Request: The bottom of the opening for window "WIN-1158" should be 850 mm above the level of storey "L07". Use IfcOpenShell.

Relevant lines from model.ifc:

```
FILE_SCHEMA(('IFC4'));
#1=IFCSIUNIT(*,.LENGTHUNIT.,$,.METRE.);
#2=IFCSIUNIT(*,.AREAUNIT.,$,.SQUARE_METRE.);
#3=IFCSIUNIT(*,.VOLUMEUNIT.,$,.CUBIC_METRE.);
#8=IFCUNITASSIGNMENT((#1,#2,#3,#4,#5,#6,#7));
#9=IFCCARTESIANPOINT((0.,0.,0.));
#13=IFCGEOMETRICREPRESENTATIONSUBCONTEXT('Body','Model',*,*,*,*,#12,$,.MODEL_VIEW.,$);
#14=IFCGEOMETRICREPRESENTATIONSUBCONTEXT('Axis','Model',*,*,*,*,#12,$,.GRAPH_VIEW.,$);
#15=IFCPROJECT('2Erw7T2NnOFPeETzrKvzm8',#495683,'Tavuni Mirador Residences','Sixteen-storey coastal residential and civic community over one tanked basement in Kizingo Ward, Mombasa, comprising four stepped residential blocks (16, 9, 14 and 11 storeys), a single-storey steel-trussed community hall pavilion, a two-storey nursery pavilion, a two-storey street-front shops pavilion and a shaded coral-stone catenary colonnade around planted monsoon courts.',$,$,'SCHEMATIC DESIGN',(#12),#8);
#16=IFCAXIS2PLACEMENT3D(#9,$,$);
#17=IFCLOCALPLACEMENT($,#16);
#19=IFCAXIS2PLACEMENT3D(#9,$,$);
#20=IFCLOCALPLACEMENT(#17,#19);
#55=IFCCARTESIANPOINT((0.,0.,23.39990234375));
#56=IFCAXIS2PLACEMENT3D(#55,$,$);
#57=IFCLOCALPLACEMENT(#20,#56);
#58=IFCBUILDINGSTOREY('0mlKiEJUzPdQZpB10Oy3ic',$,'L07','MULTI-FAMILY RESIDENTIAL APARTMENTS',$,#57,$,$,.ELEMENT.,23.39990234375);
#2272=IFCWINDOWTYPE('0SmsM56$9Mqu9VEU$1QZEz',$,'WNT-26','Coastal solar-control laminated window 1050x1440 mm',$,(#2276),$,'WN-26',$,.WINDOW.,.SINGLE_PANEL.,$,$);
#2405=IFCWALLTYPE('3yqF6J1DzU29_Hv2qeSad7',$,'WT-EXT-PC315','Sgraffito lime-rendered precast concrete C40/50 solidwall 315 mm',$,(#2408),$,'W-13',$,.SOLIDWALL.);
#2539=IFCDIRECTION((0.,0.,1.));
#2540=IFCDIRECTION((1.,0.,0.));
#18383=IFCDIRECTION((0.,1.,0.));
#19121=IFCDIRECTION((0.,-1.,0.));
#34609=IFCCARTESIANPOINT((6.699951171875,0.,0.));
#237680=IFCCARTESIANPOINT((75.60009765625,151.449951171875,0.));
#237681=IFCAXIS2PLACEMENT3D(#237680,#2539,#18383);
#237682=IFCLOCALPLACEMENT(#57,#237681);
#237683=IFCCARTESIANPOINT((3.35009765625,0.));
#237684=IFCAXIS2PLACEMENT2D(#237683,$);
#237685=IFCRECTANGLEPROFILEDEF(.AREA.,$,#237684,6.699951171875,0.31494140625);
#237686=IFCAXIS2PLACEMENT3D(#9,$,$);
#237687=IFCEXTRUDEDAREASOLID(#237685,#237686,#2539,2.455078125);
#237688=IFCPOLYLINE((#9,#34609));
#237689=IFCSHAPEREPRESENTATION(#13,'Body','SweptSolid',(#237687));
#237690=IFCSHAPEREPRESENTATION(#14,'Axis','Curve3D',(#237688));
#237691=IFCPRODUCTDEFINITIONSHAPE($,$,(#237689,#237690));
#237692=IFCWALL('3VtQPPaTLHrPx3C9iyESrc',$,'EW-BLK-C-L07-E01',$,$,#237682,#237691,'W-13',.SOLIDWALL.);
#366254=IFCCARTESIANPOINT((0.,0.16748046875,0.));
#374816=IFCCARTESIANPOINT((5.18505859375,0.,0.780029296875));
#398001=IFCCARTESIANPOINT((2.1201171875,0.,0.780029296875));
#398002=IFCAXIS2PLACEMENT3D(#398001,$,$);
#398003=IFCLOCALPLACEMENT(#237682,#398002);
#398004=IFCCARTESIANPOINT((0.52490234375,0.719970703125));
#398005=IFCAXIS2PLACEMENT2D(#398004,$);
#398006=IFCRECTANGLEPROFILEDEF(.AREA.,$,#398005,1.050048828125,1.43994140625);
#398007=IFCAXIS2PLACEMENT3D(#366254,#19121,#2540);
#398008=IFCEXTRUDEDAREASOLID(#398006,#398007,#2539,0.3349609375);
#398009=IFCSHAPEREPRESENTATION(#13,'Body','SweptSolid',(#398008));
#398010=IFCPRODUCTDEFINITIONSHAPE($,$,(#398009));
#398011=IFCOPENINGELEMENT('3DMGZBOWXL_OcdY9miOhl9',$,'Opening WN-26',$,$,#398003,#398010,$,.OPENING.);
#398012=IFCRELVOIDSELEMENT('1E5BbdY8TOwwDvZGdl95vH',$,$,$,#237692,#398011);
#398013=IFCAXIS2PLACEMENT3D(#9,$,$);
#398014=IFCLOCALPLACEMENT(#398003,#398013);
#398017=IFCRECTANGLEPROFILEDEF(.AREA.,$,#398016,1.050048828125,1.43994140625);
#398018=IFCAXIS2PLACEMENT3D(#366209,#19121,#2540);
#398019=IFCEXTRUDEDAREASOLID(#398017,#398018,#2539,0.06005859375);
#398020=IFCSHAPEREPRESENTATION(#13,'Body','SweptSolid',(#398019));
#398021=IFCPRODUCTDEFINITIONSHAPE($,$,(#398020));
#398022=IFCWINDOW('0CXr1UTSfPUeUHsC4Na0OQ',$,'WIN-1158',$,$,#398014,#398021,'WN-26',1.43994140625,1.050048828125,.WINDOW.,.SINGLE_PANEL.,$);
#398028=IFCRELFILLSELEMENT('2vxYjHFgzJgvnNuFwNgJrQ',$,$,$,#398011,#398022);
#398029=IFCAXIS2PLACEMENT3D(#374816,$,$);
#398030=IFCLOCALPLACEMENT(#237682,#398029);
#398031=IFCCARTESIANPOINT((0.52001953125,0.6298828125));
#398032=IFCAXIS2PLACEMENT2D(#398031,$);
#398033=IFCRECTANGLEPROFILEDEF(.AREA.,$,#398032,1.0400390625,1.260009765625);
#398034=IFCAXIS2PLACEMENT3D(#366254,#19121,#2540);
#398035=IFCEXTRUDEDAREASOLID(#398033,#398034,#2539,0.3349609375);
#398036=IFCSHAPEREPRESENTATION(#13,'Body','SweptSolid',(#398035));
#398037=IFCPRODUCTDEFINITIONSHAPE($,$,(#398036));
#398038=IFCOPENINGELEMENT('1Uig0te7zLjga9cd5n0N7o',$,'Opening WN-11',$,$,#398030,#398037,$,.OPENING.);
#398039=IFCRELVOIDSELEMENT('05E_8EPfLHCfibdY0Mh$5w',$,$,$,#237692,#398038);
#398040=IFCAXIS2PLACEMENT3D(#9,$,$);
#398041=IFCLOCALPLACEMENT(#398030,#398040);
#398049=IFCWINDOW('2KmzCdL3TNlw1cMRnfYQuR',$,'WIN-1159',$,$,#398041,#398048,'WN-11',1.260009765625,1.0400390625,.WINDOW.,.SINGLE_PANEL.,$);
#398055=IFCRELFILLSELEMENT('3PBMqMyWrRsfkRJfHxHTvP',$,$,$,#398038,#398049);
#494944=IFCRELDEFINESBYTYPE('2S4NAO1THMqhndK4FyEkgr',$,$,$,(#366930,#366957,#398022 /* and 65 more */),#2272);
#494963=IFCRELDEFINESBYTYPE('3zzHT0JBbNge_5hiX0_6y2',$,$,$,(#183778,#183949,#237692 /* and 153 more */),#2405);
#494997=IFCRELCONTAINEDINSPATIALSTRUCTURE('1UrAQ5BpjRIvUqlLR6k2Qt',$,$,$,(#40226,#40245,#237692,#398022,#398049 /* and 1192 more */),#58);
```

```python
import numpy as np
import ifcopenshell
import ifcopenshell.api.geometry
import ifcopenshell.geom
import ifcopenshell.util.element
import ifcopenshell.util.placement
import ifcopenshell.util.shape
import ifcopenshell.util.unit

model = ifcopenshell.open("model.ifc")
unit_scale = ifcopenshell.util.unit.calculate_unit_scale(model)

window = model.by_guid("0CXr1UTSfPUeUHsC4Na0OQ")
opening = window.FillsVoids[0].RelatingOpeningElement
storey = ifcopenshell.util.element.get_container(window, ifc_class="IfcBuildingStorey")
level = ifcopenshell.util.placement.get_local_placement(storey.ObjectPlacement)[2, 3]

# The opening's origin need not be at the sill, so measure its lowest point.
shape = ifcopenshell.geom.create_shape(ifcopenshell.geom.settings(), opening)
bottom = ifcopenshell.util.shape.get_shape_bottom_elevation(shape, shape.geometry) / unit_scale
dz = level + 0.85 / unit_scale - bottom

shift = np.array([0.0, 0.0, dz])
# The window is placed relative to its opening, so it follows when the opening moves.
matrix = ifcopenshell.util.placement.get_local_placement(opening.ObjectPlacement)
matrix[:3, 3] += shift
ifcopenshell.api.geometry.edit_object_placement(
    model, product=opening, matrix=matrix, is_si=False, should_transform_children=True
)

print(f"moved by {dz * unit_scale:+.3f} m")

model.write("model_updated.ifc")
```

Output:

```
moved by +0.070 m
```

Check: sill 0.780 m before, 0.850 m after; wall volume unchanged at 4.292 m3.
